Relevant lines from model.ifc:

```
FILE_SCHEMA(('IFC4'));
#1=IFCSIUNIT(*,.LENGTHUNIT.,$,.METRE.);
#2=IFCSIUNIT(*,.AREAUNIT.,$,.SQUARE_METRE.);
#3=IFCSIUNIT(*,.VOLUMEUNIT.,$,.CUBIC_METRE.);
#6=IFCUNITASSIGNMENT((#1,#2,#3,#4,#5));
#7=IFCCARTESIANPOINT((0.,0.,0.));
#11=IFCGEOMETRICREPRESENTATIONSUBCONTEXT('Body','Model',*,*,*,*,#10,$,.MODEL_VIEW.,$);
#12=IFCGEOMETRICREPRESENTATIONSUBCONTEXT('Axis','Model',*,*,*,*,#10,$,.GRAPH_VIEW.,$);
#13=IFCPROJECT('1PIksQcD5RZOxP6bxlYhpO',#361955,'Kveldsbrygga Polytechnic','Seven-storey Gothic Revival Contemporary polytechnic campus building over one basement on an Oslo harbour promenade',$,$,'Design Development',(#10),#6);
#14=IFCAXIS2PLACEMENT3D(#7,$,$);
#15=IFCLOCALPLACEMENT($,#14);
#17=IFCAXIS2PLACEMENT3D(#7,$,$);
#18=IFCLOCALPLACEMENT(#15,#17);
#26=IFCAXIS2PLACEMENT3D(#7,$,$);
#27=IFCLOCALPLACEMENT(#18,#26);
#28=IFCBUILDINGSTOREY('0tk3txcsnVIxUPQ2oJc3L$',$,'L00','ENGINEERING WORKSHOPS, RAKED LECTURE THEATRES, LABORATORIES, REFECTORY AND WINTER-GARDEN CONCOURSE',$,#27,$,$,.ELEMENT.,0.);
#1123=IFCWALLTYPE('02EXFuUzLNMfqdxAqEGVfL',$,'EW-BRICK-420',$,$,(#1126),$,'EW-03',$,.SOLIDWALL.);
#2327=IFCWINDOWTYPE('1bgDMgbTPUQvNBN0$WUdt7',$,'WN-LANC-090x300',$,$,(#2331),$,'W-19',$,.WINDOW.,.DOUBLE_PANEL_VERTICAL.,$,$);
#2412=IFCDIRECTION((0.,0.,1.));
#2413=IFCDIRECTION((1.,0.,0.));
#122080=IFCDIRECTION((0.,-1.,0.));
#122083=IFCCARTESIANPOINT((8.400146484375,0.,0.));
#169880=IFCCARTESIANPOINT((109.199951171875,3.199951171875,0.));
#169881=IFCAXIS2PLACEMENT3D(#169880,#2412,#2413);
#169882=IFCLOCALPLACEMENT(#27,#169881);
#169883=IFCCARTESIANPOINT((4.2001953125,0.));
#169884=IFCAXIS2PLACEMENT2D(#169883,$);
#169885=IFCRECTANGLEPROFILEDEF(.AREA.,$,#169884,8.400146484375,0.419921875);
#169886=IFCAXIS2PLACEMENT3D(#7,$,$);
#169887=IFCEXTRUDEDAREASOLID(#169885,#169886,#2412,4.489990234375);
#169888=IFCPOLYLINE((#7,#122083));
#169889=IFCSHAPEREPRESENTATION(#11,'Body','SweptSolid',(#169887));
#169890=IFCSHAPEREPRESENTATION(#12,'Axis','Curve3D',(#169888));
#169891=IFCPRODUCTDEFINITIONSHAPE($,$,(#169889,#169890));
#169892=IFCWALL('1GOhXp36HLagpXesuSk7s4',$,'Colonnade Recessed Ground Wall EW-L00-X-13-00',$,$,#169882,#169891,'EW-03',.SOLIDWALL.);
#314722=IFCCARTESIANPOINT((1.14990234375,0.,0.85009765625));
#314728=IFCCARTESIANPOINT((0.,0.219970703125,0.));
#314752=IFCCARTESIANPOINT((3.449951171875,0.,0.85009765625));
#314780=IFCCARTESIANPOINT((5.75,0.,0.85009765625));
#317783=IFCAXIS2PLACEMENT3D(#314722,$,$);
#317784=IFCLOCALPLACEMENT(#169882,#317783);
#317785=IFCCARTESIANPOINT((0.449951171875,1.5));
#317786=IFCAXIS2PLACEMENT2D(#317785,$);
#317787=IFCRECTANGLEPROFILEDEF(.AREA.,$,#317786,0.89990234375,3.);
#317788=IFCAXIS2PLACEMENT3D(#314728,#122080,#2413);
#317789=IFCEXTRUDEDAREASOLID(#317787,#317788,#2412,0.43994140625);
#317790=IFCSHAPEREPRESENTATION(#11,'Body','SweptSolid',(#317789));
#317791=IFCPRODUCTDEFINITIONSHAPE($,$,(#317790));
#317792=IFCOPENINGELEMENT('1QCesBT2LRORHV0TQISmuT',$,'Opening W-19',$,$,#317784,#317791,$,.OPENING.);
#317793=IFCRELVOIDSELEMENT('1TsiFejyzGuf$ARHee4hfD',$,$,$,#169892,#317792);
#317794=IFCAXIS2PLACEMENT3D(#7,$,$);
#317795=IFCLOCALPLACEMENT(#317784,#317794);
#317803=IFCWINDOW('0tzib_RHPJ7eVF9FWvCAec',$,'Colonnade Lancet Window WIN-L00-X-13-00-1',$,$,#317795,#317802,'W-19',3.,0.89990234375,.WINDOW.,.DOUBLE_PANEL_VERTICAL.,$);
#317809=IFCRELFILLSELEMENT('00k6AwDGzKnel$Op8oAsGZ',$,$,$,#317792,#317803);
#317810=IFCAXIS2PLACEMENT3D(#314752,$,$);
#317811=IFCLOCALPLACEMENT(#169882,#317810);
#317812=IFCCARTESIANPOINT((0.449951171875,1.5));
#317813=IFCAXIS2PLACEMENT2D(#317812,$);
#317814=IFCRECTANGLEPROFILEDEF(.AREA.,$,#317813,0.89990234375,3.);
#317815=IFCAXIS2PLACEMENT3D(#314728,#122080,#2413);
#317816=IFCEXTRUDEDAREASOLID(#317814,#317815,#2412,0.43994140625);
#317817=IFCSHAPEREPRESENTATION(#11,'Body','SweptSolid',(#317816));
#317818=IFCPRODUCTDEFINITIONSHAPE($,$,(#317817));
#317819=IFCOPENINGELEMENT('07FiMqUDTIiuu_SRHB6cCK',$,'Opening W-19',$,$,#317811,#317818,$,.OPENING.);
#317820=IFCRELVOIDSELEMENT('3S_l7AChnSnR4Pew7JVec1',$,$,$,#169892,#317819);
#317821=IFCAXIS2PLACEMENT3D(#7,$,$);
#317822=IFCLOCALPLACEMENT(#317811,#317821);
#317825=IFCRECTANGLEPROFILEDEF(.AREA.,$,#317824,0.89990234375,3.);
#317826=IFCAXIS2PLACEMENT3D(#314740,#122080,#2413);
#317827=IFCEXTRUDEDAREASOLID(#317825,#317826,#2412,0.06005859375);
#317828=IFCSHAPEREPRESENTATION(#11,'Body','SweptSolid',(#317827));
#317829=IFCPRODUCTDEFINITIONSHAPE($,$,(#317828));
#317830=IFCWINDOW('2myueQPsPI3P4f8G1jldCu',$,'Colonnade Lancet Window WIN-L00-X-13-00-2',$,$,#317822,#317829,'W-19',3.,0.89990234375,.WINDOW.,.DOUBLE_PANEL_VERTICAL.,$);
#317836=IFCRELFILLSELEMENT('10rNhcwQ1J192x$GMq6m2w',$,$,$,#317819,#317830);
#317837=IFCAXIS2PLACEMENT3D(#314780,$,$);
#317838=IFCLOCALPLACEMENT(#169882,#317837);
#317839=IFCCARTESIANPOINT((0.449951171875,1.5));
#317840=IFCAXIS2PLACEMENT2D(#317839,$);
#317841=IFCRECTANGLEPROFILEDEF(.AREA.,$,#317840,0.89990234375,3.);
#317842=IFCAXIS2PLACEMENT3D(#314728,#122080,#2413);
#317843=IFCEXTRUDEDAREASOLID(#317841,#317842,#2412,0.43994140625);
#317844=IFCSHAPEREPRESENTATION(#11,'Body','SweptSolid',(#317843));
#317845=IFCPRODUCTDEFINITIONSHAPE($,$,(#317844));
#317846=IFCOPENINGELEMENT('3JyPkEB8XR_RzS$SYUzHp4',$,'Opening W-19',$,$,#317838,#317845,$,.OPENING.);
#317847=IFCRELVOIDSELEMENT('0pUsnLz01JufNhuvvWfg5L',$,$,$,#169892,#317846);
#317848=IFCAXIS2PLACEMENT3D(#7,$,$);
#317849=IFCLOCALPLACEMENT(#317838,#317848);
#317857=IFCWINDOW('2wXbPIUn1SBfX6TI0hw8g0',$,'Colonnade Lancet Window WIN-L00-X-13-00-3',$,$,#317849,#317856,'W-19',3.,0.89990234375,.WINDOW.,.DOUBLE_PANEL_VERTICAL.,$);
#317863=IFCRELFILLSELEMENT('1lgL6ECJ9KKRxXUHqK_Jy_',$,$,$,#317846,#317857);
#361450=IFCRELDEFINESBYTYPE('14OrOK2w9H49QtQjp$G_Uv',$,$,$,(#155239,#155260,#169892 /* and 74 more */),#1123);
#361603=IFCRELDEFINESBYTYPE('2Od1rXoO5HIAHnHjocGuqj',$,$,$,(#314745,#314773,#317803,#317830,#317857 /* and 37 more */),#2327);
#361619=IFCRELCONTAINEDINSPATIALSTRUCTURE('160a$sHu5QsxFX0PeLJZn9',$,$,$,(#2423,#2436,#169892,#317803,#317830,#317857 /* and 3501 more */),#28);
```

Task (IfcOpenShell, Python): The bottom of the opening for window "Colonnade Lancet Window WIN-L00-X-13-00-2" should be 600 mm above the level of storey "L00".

```python
import numpy as np
import ifcopenshell
import ifcopenshell.api.geometry
import ifcopenshell.geom
import ifcopenshell.util.element
import ifcopenshell.util.placement
import ifcopenshell.util.shape
import ifcopenshell.util.unit

model = ifcopenshell.open("model.ifc")
unit_scale = ifcopenshell.util.unit.calculate_unit_scale(model)

window = model.by_guid("2myueQPsPI3P4f8G1jldCu")
opening = window.FillsVoids[0].RelatingOpeningElement
storey = ifcopenshell.util.element.get_container(window, ifc_class="IfcBuildingStorey")
level = ifcopenshell.util.placement.get_local_placement(storey.ObjectPlacement)[2, 3]

# The opening's origin need not be at the sill, so measure its lowest point.
shape = ifcopenshell.geom.create_shape(ifcopenshell.geom.settings(), opening)
bottom = ifcopenshell.util.shape.get_shape_bottom_elevation(shape, shape.geometry) / unit_scale
dz = level + 0.6 / unit_scale - bottom

shift = np.array([0.0, 0.0, dz])
# The window is placed relative to its opening, so it follows when the opening moves.
matrix = ifcopenshell.util.placement.get_local_placement(opening.ObjectPlacement)
matrix[:3, 3] += shift
ifcopenshell.api.geometry.edit_object_placement(
    model, product=opening, matrix=matrix, is_si=False, should_transform_children=True
)

print(f"moved by {dz * unit_scale:+.3f} m")

model.write("model_v2.ifc")
```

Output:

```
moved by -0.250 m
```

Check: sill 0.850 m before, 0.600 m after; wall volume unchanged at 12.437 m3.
